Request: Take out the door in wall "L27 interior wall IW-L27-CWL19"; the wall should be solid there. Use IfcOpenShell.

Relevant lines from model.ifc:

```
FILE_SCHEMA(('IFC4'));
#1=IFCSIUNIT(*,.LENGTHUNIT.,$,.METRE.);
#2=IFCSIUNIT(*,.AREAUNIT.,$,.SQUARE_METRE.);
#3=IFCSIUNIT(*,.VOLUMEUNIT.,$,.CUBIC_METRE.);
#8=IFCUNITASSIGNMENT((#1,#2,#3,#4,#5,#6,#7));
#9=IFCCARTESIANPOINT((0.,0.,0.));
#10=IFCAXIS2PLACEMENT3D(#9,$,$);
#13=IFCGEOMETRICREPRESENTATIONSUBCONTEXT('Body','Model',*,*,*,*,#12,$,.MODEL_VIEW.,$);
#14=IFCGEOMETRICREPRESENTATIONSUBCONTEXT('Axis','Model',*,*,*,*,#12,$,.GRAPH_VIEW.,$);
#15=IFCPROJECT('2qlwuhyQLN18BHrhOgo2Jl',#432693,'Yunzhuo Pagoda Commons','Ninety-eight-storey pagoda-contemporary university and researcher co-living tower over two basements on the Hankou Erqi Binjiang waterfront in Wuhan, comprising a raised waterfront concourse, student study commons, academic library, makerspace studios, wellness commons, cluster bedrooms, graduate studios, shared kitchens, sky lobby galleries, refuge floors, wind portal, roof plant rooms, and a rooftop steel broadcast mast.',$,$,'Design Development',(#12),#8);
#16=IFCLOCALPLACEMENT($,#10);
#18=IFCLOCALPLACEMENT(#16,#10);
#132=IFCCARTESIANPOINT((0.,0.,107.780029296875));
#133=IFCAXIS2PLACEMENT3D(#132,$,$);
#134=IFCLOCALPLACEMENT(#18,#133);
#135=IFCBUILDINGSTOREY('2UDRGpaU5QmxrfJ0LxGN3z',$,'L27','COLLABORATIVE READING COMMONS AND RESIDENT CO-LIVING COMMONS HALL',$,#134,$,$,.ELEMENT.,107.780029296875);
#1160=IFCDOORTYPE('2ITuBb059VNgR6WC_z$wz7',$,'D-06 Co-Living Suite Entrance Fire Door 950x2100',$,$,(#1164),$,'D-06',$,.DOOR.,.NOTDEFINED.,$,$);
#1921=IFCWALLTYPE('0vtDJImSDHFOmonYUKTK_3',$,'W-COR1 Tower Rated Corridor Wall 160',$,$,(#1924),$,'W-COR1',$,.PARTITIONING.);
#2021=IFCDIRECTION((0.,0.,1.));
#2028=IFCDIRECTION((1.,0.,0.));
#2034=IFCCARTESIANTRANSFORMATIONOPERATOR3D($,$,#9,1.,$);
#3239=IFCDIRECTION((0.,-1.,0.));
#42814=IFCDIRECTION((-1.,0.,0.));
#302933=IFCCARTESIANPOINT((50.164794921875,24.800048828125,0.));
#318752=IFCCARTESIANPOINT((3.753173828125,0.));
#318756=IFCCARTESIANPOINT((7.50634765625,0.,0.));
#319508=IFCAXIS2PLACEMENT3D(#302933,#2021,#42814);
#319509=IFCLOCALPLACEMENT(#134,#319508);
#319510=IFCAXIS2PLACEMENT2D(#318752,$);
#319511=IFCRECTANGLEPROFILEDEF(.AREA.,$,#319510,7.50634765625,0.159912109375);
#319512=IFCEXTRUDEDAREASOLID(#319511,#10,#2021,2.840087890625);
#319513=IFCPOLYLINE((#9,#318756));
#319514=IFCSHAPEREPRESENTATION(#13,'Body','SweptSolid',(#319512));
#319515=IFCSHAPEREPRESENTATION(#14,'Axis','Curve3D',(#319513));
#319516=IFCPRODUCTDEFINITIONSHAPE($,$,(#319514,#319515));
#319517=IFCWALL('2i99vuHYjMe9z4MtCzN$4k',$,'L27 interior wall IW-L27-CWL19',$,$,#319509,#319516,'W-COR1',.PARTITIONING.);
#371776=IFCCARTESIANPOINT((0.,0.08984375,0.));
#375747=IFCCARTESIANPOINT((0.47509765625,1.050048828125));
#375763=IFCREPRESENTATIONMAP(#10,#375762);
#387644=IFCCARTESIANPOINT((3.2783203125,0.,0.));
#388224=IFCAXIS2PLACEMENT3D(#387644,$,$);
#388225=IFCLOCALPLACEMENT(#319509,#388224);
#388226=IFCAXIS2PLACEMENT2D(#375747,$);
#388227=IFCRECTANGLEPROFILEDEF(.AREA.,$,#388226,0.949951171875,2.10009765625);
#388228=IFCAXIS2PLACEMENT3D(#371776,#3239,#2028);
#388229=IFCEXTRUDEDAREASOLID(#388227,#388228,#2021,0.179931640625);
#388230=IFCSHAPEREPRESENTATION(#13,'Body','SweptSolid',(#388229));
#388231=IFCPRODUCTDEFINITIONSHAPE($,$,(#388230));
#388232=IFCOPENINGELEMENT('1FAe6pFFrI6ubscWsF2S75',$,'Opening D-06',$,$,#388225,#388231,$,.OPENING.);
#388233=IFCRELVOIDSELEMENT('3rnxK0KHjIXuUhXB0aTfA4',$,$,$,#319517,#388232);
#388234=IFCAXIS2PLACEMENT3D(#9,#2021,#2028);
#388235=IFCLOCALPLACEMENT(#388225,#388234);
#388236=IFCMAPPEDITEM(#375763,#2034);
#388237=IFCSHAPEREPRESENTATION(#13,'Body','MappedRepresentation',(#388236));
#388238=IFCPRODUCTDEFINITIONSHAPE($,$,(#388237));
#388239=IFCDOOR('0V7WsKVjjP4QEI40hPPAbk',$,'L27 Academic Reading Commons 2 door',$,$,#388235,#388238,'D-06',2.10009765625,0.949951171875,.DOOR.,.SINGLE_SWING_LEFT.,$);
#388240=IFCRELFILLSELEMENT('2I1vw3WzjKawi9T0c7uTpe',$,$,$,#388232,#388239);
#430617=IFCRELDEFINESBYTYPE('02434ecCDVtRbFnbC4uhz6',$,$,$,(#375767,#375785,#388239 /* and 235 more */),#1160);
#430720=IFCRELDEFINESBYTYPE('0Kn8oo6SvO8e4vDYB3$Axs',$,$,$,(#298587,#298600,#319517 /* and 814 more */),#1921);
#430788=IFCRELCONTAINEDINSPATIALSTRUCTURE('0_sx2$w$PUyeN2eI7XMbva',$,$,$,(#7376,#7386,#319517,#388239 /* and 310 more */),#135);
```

```python
import ifcopenshell
import ifcopenshell.api.feature
import ifcopenshell.api.root
import ifcopenshell.geom
import ifcopenshell.util.shape

model = ifcopenshell.open("model.ifc")
settings = ifcopenshell.geom.settings()


def volume(element):
    """Net volume in cubic metres, openings subtracted."""
    shape = ifcopenshell.geom.create_shape(settings, element)
    return ifcopenshell.util.shape.get_volume(shape.geometry)


door = model.by_id(388239)
opening = door.FillsVoids[0].RelatingOpeningElement
wall = opening.VoidsElements[0].RelatingBuildingElement
before = volume(wall)

ifcopenshell.api.root.remove_product(model, product=door)
ifcopenshell.api.feature.remove_feature(model, feature=opening)

after = volume(wall)

print(f"wall volume {before:.3f} -> {after:.3f} m3")

model.write("model_rev.ifc")
```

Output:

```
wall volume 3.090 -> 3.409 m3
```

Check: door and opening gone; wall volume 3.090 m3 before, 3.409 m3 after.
